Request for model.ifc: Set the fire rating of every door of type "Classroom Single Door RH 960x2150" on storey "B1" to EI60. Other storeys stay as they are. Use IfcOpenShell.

First a look at what the model holds.

```python
import ifcopenshell
import ifcopenshell.util.element

model = ifcopenshell.open("model.ifc")
print(model.schema)
storey = next(s for s in model.by_type("IfcBuildingStorey") if s.Name == "B1")
doors = [e for e in ifcopenshell.util.element.get_decomposition(storey) if e.is_a("IfcDoor")]
seen = {}
for e in doors:
    element_type = ifcopenshell.util.element.get_type(e)
    key = (element_type.Name if element_type != e and element_type else None, ifcopenshell.util.element.get_pset(e, "Pset_DoorCommon", "FireRating"))
    seen[key] = seen.get(key, 0) + 1
for (name, value), count in sorted(seen.items(), key=str):
    print(count, "x", name, "|", value)
```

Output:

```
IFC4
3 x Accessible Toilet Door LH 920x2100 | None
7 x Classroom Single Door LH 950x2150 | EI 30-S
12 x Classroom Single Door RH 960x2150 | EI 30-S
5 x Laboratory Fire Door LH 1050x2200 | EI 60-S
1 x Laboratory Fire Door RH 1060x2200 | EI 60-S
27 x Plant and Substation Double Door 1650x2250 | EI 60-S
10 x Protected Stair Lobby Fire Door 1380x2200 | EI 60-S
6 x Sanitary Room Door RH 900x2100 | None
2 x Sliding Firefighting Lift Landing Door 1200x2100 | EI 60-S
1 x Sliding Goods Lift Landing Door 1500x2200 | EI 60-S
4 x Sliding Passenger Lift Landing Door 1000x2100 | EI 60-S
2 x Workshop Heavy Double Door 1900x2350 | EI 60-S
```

```python
import ifcopenshell
import ifcopenshell.api.pset
import ifcopenshell.util.element

model = ifcopenshell.open("model.ifc")

storey = next(s for s in model.by_type("IfcBuildingStorey") if s.Name == "B1")
doors = [e for e in ifcopenshell.util.element.get_decomposition(storey) if e.is_a("IfcDoor")]

count = 0
for e in doors:
    element_type = ifcopenshell.util.element.get_type(e)
    if element_type in (None, e) or element_type.Name != "Classroom Single Door RH 960x2150":
        continue
    # add_pset returns the element's existing set when there is one.
    pset = ifcopenshell.api.pset.add_pset(model, product=e, name="Pset_DoorCommon")
    ifcopenshell.api.pset.edit_pset(model, pset=pset, properties={"FireRating": "EI60"})
    count += 1

print(count, "doors updated")

model.write("model_rev.ifc")
```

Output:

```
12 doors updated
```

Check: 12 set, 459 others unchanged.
